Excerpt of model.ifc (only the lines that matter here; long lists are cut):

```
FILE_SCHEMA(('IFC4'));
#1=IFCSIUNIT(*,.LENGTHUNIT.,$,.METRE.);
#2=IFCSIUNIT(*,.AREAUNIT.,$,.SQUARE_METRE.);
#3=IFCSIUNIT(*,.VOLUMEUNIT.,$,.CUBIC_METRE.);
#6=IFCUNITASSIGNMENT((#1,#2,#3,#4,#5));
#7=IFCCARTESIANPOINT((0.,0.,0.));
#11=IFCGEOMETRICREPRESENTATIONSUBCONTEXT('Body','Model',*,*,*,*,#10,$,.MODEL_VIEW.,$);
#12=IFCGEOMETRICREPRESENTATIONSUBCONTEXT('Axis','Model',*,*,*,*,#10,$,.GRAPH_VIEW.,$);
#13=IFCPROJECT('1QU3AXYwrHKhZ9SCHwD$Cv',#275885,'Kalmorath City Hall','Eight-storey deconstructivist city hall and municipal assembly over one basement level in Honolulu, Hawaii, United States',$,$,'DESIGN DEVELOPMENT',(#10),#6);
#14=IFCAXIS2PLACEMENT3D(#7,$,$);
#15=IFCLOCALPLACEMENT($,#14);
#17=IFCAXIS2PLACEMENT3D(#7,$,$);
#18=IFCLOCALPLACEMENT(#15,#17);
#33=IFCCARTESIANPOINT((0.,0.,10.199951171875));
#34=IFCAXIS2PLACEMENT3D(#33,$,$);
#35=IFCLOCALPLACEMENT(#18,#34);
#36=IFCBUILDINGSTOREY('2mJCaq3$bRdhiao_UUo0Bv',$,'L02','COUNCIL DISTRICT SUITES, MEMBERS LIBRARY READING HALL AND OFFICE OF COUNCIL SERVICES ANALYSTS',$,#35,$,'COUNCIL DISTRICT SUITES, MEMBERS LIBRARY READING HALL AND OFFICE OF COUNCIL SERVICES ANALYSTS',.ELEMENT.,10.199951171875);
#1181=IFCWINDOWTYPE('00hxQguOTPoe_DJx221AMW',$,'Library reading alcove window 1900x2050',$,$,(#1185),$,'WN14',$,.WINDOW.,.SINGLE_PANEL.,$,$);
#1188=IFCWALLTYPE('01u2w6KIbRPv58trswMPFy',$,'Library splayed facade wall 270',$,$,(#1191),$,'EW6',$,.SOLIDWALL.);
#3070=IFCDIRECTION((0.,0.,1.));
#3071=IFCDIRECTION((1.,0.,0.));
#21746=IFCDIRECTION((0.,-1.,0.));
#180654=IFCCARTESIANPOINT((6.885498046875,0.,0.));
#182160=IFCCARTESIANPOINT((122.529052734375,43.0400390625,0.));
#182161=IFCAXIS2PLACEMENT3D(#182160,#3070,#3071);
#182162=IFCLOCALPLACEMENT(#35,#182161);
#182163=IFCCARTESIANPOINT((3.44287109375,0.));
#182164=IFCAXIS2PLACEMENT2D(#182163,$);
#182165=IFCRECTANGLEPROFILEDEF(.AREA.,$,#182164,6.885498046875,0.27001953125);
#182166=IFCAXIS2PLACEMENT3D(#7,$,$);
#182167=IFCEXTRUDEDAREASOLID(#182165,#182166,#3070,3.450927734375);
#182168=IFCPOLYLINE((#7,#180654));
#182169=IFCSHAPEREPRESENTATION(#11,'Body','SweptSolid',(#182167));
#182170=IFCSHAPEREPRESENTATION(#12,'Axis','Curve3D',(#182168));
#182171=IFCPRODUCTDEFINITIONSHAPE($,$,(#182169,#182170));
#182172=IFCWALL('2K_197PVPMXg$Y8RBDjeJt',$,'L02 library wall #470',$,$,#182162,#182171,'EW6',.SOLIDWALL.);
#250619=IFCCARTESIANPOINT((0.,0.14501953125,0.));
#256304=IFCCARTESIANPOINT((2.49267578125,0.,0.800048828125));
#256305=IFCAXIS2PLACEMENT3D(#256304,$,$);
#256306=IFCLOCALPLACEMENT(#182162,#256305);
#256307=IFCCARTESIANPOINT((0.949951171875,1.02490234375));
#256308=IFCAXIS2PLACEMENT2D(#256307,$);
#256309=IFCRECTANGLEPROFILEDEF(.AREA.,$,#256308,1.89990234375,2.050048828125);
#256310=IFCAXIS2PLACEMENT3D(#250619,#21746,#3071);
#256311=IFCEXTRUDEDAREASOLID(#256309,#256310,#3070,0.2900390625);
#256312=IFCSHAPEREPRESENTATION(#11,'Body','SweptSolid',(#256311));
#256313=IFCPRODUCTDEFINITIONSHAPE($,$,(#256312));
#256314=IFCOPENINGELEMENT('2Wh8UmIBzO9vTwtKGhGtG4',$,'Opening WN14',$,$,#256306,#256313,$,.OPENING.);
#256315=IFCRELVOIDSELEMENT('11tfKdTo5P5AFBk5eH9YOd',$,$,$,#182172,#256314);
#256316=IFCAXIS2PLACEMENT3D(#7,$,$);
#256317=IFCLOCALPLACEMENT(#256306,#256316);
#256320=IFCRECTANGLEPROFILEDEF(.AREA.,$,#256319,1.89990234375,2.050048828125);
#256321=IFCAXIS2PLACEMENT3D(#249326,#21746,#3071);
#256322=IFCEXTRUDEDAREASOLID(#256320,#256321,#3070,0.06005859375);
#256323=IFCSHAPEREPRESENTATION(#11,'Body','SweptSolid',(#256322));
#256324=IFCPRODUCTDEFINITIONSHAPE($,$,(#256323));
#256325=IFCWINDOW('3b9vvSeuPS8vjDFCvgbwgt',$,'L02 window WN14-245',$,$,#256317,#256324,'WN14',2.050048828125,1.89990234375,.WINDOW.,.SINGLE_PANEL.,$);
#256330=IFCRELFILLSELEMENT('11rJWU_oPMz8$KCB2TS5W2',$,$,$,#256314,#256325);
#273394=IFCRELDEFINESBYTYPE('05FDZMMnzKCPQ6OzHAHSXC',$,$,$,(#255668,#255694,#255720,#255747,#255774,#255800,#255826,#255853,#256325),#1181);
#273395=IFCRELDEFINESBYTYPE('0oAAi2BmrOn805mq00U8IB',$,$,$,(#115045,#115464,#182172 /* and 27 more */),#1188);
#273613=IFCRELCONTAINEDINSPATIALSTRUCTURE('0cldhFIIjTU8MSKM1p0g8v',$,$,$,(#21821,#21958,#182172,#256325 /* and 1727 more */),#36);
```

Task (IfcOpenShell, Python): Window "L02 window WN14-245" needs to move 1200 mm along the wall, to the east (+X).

```python
import ifcopenshell
import ifcopenshell.api.geometry
import ifcopenshell.util.placement
import ifcopenshell.util.unit

model = ifcopenshell.open("model.ifc")
unit_scale = ifcopenshell.util.unit.calculate_unit_scale(model)

window = model.by_id(256325)
opening = window.FillsVoids[0].RelatingOpeningElement
wall = opening.VoidsElements[0].RelatingBuildingElement

wall_matrix = ifcopenshell.util.placement.get_local_placement(wall.ObjectPlacement)
shift = wall_matrix[:3, 0] * 1.2 / unit_scale
before = ifcopenshell.util.placement.get_local_placement(window.ObjectPlacement)[:3, 3].copy()

# The window is placed relative to its opening, so it follows when the opening moves.
matrix = ifcopenshell.util.placement.get_local_placement(opening.ObjectPlacement)
matrix[:3, 3] += shift
ifcopenshell.api.geometry.edit_object_placement(
    model, product=opening, matrix=matrix, is_si=False, should_transform_children=True
)

after = ifcopenshell.util.placement.get_local_placement(window.ObjectPlacement)[:3, 3]
print("window moved by", (after - before).round(3) + 0.0)

model.write("model_updated.ifc")
```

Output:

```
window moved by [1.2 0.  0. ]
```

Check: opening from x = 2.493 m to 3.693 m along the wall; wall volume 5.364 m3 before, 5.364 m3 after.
